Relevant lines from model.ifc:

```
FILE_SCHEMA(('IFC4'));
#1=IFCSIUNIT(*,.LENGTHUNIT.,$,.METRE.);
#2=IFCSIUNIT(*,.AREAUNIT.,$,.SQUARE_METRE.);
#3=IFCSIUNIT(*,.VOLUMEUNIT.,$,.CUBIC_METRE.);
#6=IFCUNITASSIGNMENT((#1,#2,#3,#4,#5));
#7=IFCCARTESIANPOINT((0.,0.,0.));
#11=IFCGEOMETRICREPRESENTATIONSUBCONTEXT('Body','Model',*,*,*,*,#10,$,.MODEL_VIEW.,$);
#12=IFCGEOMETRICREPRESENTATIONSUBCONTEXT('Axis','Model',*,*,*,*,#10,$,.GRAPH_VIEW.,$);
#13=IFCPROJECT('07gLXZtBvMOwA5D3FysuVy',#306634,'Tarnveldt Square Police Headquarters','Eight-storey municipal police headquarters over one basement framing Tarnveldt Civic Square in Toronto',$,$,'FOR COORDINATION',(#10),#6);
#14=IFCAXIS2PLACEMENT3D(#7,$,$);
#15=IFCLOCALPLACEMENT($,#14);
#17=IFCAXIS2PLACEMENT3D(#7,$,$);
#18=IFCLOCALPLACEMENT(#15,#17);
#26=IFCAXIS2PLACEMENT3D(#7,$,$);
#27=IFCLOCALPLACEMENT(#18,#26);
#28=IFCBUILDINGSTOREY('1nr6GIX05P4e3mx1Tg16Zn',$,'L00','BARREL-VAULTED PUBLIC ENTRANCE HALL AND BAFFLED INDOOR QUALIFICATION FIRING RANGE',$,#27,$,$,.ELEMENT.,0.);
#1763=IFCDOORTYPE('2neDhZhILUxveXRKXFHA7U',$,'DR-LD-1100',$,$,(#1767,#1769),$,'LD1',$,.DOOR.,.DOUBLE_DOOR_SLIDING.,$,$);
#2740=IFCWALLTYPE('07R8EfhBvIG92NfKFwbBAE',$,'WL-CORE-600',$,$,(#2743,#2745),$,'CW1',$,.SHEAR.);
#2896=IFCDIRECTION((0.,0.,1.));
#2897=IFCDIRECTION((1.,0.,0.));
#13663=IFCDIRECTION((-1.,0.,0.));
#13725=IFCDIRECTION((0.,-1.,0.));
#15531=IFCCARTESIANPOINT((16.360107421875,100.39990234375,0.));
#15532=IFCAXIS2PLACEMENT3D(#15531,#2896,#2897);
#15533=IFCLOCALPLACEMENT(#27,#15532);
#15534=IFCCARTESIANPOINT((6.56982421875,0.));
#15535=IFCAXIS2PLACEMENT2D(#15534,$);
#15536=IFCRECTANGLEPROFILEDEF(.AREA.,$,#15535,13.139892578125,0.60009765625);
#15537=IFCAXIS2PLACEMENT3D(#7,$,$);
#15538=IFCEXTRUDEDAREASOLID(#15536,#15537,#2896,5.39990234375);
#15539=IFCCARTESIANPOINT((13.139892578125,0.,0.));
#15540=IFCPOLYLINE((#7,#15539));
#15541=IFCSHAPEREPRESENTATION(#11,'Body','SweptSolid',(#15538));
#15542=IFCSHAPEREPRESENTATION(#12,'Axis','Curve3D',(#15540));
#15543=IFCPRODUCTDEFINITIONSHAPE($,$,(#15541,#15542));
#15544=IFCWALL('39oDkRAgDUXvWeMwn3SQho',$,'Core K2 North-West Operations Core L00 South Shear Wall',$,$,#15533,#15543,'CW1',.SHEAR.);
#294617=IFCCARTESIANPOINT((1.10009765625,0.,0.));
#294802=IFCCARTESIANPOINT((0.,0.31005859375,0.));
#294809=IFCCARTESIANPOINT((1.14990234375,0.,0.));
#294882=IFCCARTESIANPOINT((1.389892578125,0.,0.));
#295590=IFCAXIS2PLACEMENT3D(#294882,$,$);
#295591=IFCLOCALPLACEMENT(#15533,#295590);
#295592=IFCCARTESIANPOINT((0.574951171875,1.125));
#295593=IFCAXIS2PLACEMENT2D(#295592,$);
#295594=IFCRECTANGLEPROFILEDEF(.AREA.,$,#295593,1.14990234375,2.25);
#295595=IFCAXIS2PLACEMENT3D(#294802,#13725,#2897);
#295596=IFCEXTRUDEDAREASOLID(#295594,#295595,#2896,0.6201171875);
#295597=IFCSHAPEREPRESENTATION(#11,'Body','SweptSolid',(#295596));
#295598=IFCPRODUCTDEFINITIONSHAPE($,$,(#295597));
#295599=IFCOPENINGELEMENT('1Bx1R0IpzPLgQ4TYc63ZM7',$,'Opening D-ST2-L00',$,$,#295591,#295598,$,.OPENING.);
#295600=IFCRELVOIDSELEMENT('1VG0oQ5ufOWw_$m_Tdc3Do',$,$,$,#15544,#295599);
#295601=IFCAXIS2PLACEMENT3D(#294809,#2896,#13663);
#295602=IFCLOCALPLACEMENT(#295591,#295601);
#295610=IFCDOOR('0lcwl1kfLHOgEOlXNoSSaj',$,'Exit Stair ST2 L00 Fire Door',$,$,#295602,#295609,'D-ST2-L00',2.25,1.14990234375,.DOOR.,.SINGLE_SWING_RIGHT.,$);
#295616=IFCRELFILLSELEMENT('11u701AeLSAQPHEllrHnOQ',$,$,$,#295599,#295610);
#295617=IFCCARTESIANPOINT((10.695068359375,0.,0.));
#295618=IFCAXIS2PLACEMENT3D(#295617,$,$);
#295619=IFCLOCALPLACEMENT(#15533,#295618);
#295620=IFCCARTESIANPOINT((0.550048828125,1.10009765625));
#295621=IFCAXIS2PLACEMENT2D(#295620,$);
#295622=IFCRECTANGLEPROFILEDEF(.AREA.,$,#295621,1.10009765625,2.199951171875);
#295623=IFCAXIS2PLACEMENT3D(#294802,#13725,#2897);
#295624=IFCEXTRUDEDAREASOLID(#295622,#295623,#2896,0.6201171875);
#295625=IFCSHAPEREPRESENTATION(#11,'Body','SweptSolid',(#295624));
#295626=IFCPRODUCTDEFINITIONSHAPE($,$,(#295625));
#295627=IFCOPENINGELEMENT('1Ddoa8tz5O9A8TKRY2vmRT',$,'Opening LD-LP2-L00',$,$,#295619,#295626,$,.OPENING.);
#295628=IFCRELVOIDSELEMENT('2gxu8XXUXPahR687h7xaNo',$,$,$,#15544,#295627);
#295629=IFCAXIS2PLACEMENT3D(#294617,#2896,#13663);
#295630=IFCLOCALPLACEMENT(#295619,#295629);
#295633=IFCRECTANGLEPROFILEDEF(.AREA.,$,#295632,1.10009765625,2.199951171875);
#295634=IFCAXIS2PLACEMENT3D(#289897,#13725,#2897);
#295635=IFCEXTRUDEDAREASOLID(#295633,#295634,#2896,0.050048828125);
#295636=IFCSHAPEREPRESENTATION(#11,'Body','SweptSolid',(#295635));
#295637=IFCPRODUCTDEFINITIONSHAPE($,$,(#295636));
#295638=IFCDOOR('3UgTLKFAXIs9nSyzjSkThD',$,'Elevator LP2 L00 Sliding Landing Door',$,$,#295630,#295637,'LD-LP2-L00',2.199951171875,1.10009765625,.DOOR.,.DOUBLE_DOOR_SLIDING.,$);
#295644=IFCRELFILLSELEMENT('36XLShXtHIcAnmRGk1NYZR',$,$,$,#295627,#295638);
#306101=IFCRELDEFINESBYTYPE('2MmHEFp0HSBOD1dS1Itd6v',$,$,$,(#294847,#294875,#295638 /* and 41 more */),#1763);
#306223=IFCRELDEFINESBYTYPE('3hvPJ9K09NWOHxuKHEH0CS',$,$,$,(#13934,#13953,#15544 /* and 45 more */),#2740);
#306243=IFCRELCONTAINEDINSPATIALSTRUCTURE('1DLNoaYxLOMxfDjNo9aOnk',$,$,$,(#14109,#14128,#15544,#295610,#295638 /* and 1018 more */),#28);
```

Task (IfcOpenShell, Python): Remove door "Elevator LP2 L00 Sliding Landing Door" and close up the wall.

```python
import ifcopenshell
import ifcopenshell.api.feature
import ifcopenshell.api.root
import ifcopenshell.geom
import ifcopenshell.util.shape

model = ifcopenshell.open("model.ifc")
settings = ifcopenshell.geom.settings()


def volume(element):
    """Net volume in cubic metres, openings subtracted."""
    shape = ifcopenshell.geom.create_shape(settings, element)
    return ifcopenshell.util.shape.get_volume(shape.geometry)


door = model.by_guid("3UgTLKFAXIs9nSyzjSkThD")
opening = door.FillsVoids[0].RelatingOpeningElement
wall = opening.VoidsElements[0].RelatingBuildingElement
before = volume(wall)

ifcopenshell.api.root.remove_product(model, product=door)
ifcopenshell.api.feature.remove_feature(model, feature=opening)

after = volume(wall)

print(f"wall volume {before:.3f} -> {after:.3f} m3")

model.write("model-out.ifc")
```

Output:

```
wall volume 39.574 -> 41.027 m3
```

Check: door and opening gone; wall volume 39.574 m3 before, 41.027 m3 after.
